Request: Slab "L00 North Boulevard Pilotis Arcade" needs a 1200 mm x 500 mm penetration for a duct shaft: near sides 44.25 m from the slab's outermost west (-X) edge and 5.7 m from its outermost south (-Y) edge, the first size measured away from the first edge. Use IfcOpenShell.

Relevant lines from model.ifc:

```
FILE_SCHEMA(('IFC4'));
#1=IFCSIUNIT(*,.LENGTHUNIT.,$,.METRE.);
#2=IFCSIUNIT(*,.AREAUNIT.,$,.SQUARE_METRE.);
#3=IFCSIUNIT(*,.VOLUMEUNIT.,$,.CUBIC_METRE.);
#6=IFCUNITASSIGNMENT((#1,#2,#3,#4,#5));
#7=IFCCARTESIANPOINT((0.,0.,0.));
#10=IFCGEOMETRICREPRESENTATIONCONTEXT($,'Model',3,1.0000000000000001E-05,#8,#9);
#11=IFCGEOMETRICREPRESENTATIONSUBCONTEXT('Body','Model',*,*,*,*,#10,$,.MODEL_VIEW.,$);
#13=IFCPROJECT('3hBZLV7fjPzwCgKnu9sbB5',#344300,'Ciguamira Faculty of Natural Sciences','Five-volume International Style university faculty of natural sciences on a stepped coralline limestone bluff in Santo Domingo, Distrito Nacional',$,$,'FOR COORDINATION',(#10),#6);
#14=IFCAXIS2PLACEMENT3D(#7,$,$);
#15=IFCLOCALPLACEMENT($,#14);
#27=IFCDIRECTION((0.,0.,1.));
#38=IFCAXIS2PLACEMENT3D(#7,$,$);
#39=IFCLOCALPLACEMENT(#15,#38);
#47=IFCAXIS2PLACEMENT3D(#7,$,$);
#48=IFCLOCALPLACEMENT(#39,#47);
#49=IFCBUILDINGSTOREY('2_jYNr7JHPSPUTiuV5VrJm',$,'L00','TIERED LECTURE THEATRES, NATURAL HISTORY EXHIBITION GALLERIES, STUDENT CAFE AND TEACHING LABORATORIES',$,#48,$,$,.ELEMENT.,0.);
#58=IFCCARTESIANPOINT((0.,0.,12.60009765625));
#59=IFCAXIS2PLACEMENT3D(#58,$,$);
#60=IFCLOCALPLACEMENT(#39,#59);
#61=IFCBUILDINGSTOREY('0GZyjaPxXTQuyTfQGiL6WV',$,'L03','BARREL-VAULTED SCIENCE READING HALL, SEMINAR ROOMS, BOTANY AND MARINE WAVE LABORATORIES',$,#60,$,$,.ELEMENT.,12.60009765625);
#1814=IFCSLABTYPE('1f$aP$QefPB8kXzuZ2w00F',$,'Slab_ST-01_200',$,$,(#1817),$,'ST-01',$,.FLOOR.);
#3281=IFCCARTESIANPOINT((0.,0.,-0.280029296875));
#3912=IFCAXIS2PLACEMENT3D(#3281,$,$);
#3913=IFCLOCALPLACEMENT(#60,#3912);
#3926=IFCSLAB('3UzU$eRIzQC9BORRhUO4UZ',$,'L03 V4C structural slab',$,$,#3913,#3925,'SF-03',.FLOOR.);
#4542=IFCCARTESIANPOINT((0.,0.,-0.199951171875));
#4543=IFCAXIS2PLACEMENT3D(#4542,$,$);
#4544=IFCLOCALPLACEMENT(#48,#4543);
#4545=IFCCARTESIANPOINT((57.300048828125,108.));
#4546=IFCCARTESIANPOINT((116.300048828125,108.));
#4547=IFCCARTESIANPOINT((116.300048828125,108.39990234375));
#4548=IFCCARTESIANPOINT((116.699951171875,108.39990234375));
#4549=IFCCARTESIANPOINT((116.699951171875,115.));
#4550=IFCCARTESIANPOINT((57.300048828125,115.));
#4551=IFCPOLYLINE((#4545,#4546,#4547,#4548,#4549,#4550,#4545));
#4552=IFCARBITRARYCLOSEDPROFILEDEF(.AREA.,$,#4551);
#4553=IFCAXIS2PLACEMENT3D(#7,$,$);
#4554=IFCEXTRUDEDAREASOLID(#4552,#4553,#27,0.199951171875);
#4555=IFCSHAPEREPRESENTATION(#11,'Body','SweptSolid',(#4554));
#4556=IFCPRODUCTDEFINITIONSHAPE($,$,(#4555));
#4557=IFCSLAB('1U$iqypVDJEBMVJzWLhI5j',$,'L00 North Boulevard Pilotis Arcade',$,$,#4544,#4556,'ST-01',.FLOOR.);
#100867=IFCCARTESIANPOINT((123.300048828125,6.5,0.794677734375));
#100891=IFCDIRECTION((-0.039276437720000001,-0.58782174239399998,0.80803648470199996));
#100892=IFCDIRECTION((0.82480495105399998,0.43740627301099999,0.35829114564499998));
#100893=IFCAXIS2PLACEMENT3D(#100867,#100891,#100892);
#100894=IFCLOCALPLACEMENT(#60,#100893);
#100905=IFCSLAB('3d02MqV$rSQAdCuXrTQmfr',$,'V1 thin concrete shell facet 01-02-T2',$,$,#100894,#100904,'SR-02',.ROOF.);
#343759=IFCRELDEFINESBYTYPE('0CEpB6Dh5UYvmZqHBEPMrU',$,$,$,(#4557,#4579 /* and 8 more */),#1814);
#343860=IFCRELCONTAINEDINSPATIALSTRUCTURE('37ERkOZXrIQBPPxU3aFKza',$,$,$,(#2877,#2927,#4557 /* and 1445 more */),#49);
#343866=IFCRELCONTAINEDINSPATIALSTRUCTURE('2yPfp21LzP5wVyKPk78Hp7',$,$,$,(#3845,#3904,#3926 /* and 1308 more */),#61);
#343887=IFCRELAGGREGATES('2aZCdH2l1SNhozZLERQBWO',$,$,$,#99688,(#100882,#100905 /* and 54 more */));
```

```python
import numpy as np
import ifcopenshell
import ifcopenshell.api.feature
import ifcopenshell.api.geometry
import ifcopenshell.api.root
import ifcopenshell.geom
import ifcopenshell.util.placement
import ifcopenshell.util.representation
import ifcopenshell.util.shape
import ifcopenshell.util.unit

model = ifcopenshell.open("model.ifc")
unit_scale = ifcopenshell.util.unit.calculate_unit_scale(model)
settings = ifcopenshell.geom.settings()


def volume(element):
    """Net volume in cubic metres, openings subtracted."""
    shape = ifcopenshell.geom.create_shape(settings, element)
    return ifcopenshell.util.shape.get_volume(shape.geometry)


slab = model.by_guid("1U$iqypVDJEBMVJzWLhI5j")
before = volume(slab)

# Extent in the slab's own axes, in metres. The edges named are its -X and -Y sides.
slab_shape = ifcopenshell.geom.create_shape(settings, slab)
vertices = ifcopenshell.util.shape.get_vertices(slab_shape.geometry)
x_min, y_min, bottom = vertices.min(axis=0)
top = vertices[:, 2].max()

opening = ifcopenshell.api.root.create_entity(model, ifc_class="IfcOpeningElement", name="Duct shaft opening", predefined_type="OPENING")
context = ifcopenshell.util.representation.get_context(model, "Model", "Body", "MODEL_VIEW")
width, depth = 1.2, 0.5
outline = [(0.0, 0.0), (width, 0.0), (width, depth), (0.0, depth), (0.0, 0.0)]
# Overshoot both faces by 50 mm so the cut is clean.
shape = ifcopenshell.api.geometry.add_slab_representation(
    model, context=context, depth=top - bottom + 0.1, polyline=outline
)
ifcopenshell.api.geometry.assign_representation(model, product=opening, representation=shape)

matrix = ifcopenshell.util.placement.get_local_placement(slab.ObjectPlacement)
matrix[:, 3] = matrix @ np.append(np.array([x_min + 44.25, y_min + 5.7, bottom - 0.05]) / unit_scale, 1.0)
ifcopenshell.api.geometry.edit_object_placement(model, product=opening, matrix=matrix, is_si=False)
ifcopenshell.api.feature.add_feature(model, feature=opening, element=slab)

after = volume(slab)

print(f"slab volume {before:.3f} -> {after:.3f} m3")

model.write("model_edited.ifc")
```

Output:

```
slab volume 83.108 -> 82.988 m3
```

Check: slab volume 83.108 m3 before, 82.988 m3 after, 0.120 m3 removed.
